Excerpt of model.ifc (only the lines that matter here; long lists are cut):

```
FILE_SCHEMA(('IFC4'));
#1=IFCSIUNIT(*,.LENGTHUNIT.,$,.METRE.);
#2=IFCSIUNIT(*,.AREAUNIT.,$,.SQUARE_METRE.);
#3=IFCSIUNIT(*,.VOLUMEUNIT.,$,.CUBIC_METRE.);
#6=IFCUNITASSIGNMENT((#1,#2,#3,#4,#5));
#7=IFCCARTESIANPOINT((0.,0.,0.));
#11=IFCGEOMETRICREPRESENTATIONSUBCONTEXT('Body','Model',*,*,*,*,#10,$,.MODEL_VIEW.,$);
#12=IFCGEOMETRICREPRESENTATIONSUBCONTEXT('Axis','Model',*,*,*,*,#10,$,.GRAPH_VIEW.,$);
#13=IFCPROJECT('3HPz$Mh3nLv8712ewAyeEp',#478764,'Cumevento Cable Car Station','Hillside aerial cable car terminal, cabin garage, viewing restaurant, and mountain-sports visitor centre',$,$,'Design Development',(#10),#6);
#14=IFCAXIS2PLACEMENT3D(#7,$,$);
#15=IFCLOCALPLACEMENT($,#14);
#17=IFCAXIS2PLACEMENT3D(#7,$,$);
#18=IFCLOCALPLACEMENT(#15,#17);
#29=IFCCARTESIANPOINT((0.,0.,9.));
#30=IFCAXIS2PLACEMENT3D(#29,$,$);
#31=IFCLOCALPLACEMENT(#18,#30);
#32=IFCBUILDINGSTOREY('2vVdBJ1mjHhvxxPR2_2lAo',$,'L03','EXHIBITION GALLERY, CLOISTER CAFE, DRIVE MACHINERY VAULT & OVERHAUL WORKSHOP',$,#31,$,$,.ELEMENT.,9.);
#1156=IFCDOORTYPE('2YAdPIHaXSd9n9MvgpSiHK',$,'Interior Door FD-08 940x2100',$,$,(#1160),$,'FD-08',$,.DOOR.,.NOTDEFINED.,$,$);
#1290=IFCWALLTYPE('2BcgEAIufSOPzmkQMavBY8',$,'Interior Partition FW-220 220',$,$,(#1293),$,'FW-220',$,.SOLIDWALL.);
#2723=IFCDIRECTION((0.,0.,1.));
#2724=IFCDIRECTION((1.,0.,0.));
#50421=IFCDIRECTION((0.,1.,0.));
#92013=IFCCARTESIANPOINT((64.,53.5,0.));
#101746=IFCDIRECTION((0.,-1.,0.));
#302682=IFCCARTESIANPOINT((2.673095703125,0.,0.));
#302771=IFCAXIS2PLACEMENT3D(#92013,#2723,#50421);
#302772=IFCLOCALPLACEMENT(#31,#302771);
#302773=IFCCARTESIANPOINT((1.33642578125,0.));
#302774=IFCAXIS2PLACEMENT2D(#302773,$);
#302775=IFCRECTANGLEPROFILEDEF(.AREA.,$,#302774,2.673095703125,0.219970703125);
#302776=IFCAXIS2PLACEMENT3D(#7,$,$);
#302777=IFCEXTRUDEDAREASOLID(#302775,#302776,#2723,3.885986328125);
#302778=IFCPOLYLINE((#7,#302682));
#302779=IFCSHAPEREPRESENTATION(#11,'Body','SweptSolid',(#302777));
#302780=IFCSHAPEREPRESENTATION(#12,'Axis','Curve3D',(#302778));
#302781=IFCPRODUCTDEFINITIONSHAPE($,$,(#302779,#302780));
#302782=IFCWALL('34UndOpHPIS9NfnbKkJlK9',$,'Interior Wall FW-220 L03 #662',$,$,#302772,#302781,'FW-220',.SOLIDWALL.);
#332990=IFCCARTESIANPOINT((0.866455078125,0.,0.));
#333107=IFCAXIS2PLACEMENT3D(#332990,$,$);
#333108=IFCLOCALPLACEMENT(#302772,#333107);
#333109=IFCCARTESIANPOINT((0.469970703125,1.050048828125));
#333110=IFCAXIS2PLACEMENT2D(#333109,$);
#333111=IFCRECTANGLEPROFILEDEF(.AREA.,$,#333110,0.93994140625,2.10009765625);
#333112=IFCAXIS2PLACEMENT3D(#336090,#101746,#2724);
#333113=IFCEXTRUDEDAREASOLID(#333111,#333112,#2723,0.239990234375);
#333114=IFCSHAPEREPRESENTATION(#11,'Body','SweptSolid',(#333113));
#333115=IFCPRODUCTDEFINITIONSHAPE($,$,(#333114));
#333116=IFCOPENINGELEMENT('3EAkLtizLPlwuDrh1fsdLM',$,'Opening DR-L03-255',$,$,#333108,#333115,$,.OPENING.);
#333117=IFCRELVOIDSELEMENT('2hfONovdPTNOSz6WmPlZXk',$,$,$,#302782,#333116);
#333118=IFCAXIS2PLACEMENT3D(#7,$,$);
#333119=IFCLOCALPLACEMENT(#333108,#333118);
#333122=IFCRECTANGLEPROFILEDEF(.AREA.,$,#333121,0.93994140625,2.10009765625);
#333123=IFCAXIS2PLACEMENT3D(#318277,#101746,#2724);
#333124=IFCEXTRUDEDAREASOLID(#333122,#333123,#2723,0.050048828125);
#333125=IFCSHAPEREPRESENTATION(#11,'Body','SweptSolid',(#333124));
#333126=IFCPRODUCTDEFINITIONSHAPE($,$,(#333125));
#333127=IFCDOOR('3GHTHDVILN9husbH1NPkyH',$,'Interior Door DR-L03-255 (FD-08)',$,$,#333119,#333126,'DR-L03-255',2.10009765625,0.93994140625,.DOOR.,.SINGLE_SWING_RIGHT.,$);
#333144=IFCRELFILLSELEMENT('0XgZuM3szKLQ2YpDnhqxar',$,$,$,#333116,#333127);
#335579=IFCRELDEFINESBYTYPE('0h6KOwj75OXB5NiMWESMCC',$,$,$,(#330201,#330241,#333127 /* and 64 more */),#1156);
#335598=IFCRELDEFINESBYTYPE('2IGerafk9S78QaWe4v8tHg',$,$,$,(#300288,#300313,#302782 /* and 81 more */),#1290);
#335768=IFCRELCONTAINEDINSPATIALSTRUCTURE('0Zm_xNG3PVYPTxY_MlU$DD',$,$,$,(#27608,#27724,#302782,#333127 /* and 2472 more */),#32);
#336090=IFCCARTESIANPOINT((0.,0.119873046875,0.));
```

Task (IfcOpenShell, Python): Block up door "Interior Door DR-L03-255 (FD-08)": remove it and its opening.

```python
import ifcopenshell
import ifcopenshell.api.feature
import ifcopenshell.api.root
import ifcopenshell.geom
import ifcopenshell.util.shape

model = ifcopenshell.open("model.ifc")
settings = ifcopenshell.geom.settings()


def volume(element):
    """Net volume in cubic metres, openings subtracted."""
    shape = ifcopenshell.geom.create_shape(settings, element)
    return ifcopenshell.util.shape.get_volume(shape.geometry)


door = model.by_id(333127)
opening = door.FillsVoids[0].RelatingOpeningElement
wall = opening.VoidsElements[0].RelatingBuildingElement
before = volume(wall)

ifcopenshell.api.root.remove_product(model, product=door)
ifcopenshell.api.feature.remove_feature(model, feature=opening)

after = volume(wall)

print(f"wall volume {before:.3f} -> {after:.3f} m3")

model.write("model_updated.ifc")
```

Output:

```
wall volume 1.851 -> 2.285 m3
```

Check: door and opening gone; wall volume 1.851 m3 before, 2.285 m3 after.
